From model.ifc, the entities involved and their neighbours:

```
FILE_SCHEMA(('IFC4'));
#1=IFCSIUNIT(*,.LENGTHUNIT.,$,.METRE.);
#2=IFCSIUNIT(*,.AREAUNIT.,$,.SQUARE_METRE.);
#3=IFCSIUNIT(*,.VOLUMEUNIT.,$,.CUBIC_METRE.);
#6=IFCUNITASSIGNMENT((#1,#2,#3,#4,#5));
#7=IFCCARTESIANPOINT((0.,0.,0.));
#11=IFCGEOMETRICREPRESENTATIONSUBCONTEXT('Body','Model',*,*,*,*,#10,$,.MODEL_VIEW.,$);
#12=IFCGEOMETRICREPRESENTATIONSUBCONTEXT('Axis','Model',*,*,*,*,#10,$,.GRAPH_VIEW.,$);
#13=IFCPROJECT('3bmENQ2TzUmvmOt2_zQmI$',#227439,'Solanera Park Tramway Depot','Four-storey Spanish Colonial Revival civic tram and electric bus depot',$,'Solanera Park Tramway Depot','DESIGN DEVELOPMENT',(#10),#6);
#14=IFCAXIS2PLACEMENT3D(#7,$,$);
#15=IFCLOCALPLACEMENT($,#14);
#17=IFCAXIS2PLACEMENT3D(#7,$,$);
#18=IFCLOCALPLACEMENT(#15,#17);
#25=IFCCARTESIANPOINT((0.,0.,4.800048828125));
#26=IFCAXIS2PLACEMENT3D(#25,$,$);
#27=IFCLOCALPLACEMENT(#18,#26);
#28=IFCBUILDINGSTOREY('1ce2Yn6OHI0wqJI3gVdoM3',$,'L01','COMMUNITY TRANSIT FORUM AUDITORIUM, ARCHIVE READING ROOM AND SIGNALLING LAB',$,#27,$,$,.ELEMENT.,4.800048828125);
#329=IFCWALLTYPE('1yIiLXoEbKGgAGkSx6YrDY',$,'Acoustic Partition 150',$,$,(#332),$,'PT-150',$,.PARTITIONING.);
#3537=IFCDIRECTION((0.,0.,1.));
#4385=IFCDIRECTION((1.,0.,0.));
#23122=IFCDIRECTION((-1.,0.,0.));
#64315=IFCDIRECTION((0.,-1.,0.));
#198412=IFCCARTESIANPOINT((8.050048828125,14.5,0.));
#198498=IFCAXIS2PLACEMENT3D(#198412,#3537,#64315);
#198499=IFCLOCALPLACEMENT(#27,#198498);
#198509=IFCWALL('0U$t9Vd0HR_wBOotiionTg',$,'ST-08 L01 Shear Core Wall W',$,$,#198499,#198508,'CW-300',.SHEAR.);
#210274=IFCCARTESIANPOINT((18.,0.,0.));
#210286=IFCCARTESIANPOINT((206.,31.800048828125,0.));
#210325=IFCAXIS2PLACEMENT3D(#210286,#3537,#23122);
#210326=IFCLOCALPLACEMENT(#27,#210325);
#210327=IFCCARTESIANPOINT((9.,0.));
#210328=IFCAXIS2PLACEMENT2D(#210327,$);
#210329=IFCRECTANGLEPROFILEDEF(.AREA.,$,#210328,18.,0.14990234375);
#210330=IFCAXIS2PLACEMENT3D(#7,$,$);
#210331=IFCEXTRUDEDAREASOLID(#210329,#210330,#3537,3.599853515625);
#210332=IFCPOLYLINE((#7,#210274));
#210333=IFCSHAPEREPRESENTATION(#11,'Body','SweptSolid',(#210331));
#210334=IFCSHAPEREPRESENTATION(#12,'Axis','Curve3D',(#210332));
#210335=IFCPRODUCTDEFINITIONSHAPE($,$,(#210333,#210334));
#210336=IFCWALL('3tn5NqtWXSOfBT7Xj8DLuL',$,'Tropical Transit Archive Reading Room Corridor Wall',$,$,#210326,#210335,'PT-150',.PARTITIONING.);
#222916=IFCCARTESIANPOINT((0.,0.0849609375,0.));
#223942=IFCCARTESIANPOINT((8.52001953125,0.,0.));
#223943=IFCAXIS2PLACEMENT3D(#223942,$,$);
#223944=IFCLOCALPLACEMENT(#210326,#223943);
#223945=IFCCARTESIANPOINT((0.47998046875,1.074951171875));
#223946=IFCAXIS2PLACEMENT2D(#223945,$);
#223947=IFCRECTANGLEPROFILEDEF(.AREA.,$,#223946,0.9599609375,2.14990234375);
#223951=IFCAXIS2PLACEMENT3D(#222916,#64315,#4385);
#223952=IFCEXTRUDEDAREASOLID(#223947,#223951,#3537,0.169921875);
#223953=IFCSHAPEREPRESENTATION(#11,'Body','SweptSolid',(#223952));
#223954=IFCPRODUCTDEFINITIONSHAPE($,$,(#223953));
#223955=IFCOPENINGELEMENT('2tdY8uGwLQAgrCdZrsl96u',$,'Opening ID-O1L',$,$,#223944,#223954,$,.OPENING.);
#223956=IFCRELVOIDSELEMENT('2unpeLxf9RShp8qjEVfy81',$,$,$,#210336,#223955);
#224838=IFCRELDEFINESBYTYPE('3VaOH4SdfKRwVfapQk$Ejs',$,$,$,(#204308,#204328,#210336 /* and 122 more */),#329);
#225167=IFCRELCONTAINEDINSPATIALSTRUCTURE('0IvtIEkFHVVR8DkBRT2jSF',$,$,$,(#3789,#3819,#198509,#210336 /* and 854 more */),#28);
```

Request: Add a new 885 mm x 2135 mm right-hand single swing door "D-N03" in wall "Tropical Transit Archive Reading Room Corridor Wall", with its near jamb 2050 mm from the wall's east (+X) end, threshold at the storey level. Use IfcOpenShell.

```python
import numpy as np
import ifcopenshell
import ifcopenshell.api.feature
import ifcopenshell.api.geometry
import ifcopenshell.api.root
import ifcopenshell.api.spatial
import ifcopenshell.geom
import ifcopenshell.util.element
import ifcopenshell.util.placement
import ifcopenshell.util.representation
import ifcopenshell.util.shape
import ifcopenshell.util.unit

model = ifcopenshell.open("model.ifc")
unit_scale = ifcopenshell.util.unit.calculate_unit_scale(model)
settings = ifcopenshell.geom.settings()


def volume(element):
    """Net volume in cubic metres, openings subtracted."""
    shape = ifcopenshell.geom.create_shape(settings, element)
    return ifcopenshell.util.shape.get_volume(shape.geometry)


wall = model.by_id(210336)
storey = ifcopenshell.util.element.get_container(wall, ifc_class="IfcBuildingStorey")
context = ifcopenshell.util.representation.get_context(model, "Model", "Body", "MODEL_VIEW")
before = volume(wall)

width, height, from_end, sill = 0.885, 2.135, 2.05, 0.0  # metres

# The wall runs along its own X axis, and the end named is its -X end.
wall_shape = ifcopenshell.geom.create_shape(settings, wall)
x, y, z = ifcopenshell.util.shape.get_vertices(wall_shape.geometry).T
start = x.min() + from_end
face, thickness = float(y.min()), float(y.max() - y.min())
wall_matrix = ifcopenshell.util.placement.get_local_placement(wall.ObjectPlacement)
level = ifcopenshell.util.placement.get_local_placement(storey.ObjectPlacement)[2, 3]


def in_wall(x, y):
    """Placement at x, y metres in the wall's axes, at sill height."""
    matrix = wall_matrix.copy()
    matrix[:, 3] = wall_matrix @ np.array([x / unit_scale, y / unit_scale, 0.0, 1.0])
    matrix[2, 3] = level + sill / unit_scale
    return matrix


# Opening: a box that overshoots both wall faces by 50 mm.
opening = ifcopenshell.api.root.create_entity(model, ifc_class="IfcOpeningElement", predefined_type="OPENING")
box = ifcopenshell.api.geometry.add_wall_representation(
    model, context=context, length=width, height=height, thickness=thickness + 0.1
)
ifcopenshell.api.geometry.assign_representation(model, product=opening, representation=box)
ifcopenshell.api.geometry.edit_object_placement(model, product=opening, matrix=in_wall(start, face - 0.05), is_si=False)
ifcopenshell.api.feature.add_feature(model, feature=opening, element=wall)

door = ifcopenshell.api.root.create_entity(model, ifc_class="IfcDoor", name="D-N03", predefined_type="DOOR")
door.OverallWidth, door.OverallHeight = width / unit_scale, height / unit_scale
door.OperationType = "SINGLE_SWING_RIGHT"
body = ifcopenshell.api.geometry.add_door_representation(
    model,
    context=context,
    overall_width=door.OverallWidth,
    overall_height=door.OverallHeight,
    operation_type="SINGLE_SWING_RIGHT",
    lining_properties={"LiningDepth": thickness / unit_scale, "ThresholdDepth": thickness / unit_scale},
)
ifcopenshell.api.geometry.assign_representation(model, product=door, representation=body)
ifcopenshell.api.spatial.assign_container(model, products=[door], relating_structure=storey)
ifcopenshell.api.feature.add_filling(model, opening=opening, element=door)

# The lining spans the wall, so the door starts at the wall face.
ifcopenshell.api.geometry.edit_object_placement(model, product=door, matrix=in_wall(start, face), is_si=False)

after = volume(wall)

print(f"wall volume {before:.3f} -> {after:.3f} m3")

model.write("model_v2.ifc")
```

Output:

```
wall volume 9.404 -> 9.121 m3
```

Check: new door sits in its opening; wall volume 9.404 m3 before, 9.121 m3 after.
